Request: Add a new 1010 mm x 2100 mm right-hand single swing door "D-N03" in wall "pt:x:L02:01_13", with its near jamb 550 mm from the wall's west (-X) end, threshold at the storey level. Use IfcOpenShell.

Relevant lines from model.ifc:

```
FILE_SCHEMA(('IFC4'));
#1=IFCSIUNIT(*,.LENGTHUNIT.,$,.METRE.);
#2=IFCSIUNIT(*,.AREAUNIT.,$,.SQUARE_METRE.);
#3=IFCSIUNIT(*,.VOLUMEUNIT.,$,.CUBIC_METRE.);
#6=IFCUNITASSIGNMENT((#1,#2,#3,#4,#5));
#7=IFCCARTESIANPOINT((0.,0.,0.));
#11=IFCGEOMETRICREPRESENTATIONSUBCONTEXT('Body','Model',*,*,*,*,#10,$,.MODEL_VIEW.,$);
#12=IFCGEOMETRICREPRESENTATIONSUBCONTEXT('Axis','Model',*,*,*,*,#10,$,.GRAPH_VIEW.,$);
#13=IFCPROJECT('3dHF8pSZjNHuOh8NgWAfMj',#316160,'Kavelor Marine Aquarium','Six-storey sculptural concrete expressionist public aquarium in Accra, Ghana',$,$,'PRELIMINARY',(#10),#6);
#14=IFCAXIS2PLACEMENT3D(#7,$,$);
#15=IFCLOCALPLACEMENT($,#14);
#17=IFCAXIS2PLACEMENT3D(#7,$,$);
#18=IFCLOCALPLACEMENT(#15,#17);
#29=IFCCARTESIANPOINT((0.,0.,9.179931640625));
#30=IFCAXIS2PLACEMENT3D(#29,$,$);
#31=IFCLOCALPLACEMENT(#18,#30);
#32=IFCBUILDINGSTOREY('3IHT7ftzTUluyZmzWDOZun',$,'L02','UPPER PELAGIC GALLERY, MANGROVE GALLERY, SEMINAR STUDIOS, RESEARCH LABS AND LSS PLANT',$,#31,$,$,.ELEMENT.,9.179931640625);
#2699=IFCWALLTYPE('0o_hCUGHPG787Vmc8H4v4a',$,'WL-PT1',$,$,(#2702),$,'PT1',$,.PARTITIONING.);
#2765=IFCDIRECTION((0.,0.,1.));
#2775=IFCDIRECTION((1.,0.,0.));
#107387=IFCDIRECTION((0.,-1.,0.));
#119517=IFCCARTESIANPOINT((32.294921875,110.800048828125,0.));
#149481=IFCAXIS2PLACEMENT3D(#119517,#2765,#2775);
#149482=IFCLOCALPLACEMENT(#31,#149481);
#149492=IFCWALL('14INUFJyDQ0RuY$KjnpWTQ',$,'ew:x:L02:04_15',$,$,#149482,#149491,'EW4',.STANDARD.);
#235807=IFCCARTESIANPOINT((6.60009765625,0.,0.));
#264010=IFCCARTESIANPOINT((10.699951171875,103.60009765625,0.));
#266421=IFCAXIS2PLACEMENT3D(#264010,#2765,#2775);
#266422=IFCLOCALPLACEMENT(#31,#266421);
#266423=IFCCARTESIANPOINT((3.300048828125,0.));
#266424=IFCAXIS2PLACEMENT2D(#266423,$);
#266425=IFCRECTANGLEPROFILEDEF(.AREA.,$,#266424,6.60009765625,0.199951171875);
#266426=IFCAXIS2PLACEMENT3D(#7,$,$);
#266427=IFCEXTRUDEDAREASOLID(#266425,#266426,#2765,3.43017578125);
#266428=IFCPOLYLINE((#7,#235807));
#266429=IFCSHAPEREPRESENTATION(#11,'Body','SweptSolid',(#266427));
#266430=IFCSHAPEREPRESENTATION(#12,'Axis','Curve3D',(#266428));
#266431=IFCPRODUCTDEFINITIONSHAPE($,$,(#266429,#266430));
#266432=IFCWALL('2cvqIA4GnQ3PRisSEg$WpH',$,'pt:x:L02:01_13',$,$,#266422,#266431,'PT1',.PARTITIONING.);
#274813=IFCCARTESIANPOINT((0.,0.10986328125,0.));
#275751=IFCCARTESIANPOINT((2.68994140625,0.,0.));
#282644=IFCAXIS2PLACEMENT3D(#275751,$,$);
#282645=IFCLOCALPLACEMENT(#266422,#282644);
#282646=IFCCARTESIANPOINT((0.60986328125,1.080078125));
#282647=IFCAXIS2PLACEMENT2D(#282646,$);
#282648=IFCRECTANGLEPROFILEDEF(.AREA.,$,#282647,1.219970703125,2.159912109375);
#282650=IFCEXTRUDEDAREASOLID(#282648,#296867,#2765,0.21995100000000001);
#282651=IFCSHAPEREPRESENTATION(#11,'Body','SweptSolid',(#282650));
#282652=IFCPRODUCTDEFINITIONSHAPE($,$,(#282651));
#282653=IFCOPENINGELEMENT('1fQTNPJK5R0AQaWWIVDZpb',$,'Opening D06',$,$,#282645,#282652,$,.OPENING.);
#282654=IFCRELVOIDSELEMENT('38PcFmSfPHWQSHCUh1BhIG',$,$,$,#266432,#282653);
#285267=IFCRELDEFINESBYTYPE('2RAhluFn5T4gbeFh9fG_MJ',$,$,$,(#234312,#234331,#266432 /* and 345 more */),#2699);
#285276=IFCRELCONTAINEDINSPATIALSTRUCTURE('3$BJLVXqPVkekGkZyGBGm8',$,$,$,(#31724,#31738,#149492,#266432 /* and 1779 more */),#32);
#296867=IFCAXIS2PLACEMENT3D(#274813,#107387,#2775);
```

```python
import numpy as np
import ifcopenshell
import ifcopenshell.api.feature
import ifcopenshell.api.geometry
import ifcopenshell.api.root
import ifcopenshell.api.spatial
import ifcopenshell.geom
import ifcopenshell.util.element
import ifcopenshell.util.placement
import ifcopenshell.util.representation
import ifcopenshell.util.shape
import ifcopenshell.util.unit

model = ifcopenshell.open("model.ifc")
unit_scale = ifcopenshell.util.unit.calculate_unit_scale(model)
settings = ifcopenshell.geom.settings()


def volume(element):
    """Net volume in cubic metres, openings subtracted."""
    shape = ifcopenshell.geom.create_shape(settings, element)
    return ifcopenshell.util.shape.get_volume(shape.geometry)


wall = model.by_guid("2cvqIA4GnQ3PRisSEg$WpH")
storey = ifcopenshell.util.element.get_container(wall, ifc_class="IfcBuildingStorey")
context = ifcopenshell.util.representation.get_context(model, "Model", "Body", "MODEL_VIEW")
before = volume(wall)

width, height, from_end, sill = 1.01, 2.1, 0.55, 0.0  # metres

# The wall runs along its own X axis, and the end named is its -X end.
wall_shape = ifcopenshell.geom.create_shape(settings, wall)
x, y, z = ifcopenshell.util.shape.get_vertices(wall_shape.geometry).T
start = x.min() + from_end
face, thickness = float(y.min()), float(y.max() - y.min())
wall_matrix = ifcopenshell.util.placement.get_local_placement(wall.ObjectPlacement)
level = ifcopenshell.util.placement.get_local_placement(storey.ObjectPlacement)[2, 3]


def in_wall(x, y):
    """Placement at x, y metres in the wall's axes, at sill height."""
    matrix = wall_matrix.copy()
    matrix[:, 3] = wall_matrix @ np.array([x / unit_scale, y / unit_scale, 0.0, 1.0])
    matrix[2, 3] = level + sill / unit_scale
    return matrix


# Opening: a box that overshoots both wall faces by 50 mm.
opening = ifcopenshell.api.root.create_entity(model, ifc_class="IfcOpeningElement", predefined_type="OPENING")
box = ifcopenshell.api.geometry.add_wall_representation(
    model, context=context, length=width, height=height, thickness=thickness + 0.1
)
ifcopenshell.api.geometry.assign_representation(model, product=opening, representation=box)
ifcopenshell.api.geometry.edit_object_placement(model, product=opening, matrix=in_wall(start, face - 0.05), is_si=False)
ifcopenshell.api.feature.add_feature(model, feature=opening, element=wall)

door = ifcopenshell.api.root.create_entity(model, ifc_class="IfcDoor", name="D-N03", predefined_type="DOOR")
door.OverallWidth, door.OverallHeight = width / unit_scale, height / unit_scale
door.OperationType = "SINGLE_SWING_RIGHT"
body = ifcopenshell.api.geometry.add_door_representation(
    model,
    context=context,
    overall_width=door.OverallWidth,
    overall_height=door.OverallHeight,
    operation_type="SINGLE_SWING_RIGHT",
    lining_properties={"LiningDepth": thickness / unit_scale, "ThresholdDepth": thickness / unit_scale},
)
ifcopenshell.api.geometry.assign_representation(model, product=door, representation=body)
ifcopenshell.api.spatial.assign_container(model, products=[door], relating_structure=storey)
ifcopenshell.api.feature.add_filling(model, opening=opening, element=door)

# The lining spans the wall, so the door starts at the wall face.
ifcopenshell.api.geometry.edit_object_placement(model, product=door, matrix=in_wall(start, face), is_si=False)

after = volume(wall)

print(f"wall volume {before:.3f} -> {after:.3f} m3")

model.write("model-out.ifc")
```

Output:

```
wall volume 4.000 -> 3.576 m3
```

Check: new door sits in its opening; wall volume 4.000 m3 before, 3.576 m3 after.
